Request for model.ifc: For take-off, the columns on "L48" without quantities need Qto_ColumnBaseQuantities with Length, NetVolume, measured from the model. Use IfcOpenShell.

First a look at what the model holds.

```python
import ifcopenshell
import ifcopenshell.util.element
import ifcopenshell.util.unit

model = ifcopenshell.open("model.ifc")
print(model.schema)
for unit_type in ("LENGTHUNIT", "AREAUNIT", "VOLUMEUNIT"):
    print(unit_type, ifcopenshell.util.unit.calculate_unit_scale(model, unit_type))
storey = next(s for s in model.by_type("IfcBuildingStorey") if s.Name == "L48")
columns = [e for e in ifcopenshell.util.element.get_decomposition(storey) if e.is_a("IfcColumn")]
for e in sorted(columns, key=lambda e: e.id()):
    print(e.id(), e.is_a(), e.Name, list(ifcopenshell.util.element.get_psets(e, qtos_only=True)), sep=" | ")
```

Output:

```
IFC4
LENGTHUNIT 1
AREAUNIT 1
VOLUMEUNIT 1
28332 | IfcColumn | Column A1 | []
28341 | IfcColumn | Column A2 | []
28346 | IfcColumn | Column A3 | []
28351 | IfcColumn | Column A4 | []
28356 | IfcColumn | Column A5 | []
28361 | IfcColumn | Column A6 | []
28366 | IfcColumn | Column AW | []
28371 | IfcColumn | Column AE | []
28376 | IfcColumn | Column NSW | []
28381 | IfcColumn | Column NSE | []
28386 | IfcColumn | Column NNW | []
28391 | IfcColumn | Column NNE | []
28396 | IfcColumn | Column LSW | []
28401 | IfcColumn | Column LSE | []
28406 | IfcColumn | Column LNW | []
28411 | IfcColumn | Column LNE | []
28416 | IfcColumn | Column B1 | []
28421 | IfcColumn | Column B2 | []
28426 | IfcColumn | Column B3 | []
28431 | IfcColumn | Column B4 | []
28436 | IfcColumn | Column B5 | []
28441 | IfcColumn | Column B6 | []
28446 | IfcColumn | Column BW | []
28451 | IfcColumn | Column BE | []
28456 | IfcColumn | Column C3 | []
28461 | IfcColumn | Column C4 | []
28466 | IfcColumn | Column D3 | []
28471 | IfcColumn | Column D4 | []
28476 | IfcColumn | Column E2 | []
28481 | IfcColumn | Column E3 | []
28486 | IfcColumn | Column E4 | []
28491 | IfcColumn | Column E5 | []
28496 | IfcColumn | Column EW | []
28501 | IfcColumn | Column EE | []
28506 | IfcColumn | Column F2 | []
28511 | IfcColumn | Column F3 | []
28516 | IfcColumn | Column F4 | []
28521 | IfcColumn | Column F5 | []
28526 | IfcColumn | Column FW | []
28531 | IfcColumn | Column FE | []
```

```python
import ifcopenshell
import ifcopenshell.api.pset
import ifcopenshell.geom
import ifcopenshell.util.element
import ifcopenshell.util.shape
import ifcopenshell.util.unit

model = ifcopenshell.open("model.ifc")
unit_scale = ifcopenshell.util.unit.calculate_unit_scale(model)
volume_scale = ifcopenshell.util.unit.calculate_unit_scale(model, "VOLUMEUNIT")
settings = ifcopenshell.geom.settings()

storey = next(s for s in model.by_type("IfcBuildingStorey") if s.Name == "L48")
columns = [e for e in ifcopenshell.util.element.get_decomposition(storey) if e.is_a("IfcColumn")]

for e in sorted(columns, key=lambda e: e.id()):
    if ifcopenshell.util.element.get_psets(e, qtos_only=True, should_inherit=False):
        continue
    # Geometry comes back in metres, in the element's own axes.
    shape = ifcopenshell.geom.create_shape(settings, e)
    values = {
        "Length": ifcopenshell.util.shape.get_z(shape.geometry) / unit_scale,
        "NetVolume": ifcopenshell.util.shape.get_volume(shape.geometry) / volume_scale,
    }
    qto = ifcopenshell.api.pset.add_qto(model, product=e, name="Qto_ColumnBaseQuantities")
    ifcopenshell.api.pset.edit_qto(model, qto=qto, properties=values)
    print(e.id(), {k: round(v, 3) for k, v in values.items()})

model.write("model_edited.ifc")
```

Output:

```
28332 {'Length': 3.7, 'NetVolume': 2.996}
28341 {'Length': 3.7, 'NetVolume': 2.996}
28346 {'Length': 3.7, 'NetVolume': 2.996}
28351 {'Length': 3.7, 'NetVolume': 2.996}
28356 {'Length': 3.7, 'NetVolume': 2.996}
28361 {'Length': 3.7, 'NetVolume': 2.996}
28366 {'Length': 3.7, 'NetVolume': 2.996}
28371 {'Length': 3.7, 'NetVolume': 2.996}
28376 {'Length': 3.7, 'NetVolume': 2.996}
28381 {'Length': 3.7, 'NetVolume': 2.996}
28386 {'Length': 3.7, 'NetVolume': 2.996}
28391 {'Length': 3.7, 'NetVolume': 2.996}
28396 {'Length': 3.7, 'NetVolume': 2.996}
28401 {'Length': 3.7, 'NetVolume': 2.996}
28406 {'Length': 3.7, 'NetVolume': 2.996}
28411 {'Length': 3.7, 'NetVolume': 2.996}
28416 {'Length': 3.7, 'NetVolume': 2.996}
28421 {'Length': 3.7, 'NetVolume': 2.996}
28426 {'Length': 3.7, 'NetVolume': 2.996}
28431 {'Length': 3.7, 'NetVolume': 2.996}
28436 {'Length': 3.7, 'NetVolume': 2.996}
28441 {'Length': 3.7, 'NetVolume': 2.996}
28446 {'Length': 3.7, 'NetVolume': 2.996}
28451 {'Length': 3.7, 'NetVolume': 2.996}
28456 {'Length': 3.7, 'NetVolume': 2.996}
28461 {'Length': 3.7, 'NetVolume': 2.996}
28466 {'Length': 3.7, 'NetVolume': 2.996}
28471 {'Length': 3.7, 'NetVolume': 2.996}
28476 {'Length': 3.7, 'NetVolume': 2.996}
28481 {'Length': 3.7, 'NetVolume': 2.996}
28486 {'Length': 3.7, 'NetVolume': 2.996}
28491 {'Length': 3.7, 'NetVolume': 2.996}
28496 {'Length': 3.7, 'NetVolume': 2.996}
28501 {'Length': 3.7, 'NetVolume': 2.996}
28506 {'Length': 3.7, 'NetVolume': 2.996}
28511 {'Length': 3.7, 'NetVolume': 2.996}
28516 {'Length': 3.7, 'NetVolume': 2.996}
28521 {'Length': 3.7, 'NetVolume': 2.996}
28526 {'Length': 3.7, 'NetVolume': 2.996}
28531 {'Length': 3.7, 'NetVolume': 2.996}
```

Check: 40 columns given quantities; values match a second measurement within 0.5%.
